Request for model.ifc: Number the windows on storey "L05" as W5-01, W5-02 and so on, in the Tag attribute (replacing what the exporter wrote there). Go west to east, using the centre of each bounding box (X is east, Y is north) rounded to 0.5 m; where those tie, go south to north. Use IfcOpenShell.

First a look at what the model holds.

```python
import ifcopenshell
import ifcopenshell.util.element
import ifcopenshell.util.placement

model = ifcopenshell.open("model.ifc")
print(model.schema)
storey = next(s for s in model.by_type("IfcBuildingStorey") if s.Name == "L05")
windows = [e for e in ifcopenshell.util.element.get_decomposition(storey) if e.is_a("IfcWindow")]
for e in sorted(windows, key=lambda e: e.id()):
    origin = ifcopenshell.util.placement.get_local_placement(e.ObjectPlacement)[:3, 3]
    print(e.id(), e.Tag, e.Name, origin.round(2) + 0.0, sep=" | ")
```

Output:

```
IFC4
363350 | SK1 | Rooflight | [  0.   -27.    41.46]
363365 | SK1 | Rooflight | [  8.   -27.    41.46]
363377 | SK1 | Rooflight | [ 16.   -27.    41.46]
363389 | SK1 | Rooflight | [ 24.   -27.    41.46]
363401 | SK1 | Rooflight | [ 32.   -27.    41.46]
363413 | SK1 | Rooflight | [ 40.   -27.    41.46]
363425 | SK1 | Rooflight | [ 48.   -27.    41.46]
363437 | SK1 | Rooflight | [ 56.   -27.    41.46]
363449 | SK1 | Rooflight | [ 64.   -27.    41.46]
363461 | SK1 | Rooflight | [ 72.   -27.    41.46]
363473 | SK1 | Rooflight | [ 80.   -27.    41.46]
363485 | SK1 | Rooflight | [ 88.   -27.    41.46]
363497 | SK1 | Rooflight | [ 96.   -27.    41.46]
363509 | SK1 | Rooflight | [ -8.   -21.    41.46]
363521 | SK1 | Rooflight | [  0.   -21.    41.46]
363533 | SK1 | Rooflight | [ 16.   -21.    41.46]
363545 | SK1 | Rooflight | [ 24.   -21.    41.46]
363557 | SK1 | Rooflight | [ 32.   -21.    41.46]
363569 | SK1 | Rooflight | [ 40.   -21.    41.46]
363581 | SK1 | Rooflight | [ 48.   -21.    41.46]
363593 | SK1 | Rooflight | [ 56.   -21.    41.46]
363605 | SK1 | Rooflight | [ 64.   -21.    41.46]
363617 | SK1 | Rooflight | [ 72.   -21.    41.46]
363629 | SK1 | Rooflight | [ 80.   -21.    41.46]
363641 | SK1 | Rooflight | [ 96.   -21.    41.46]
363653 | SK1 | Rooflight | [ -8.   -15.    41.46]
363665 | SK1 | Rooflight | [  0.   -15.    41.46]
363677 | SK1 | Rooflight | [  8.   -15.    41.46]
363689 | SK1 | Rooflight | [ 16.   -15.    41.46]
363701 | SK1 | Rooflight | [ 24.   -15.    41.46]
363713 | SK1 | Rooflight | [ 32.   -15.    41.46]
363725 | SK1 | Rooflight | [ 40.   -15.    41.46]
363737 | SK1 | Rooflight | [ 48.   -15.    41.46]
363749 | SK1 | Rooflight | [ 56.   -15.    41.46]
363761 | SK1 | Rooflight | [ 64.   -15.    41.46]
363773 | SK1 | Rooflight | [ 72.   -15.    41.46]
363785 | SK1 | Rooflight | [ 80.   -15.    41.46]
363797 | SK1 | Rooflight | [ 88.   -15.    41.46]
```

```python
import ifcopenshell
import ifcopenshell.geom
import ifcopenshell.util.element
import ifcopenshell.util.shape

model = ifcopenshell.open("model.ifc")
settings = ifcopenshell.geom.settings()
settings.set("use-world-coords", True)


def centre(element):
    shape = ifcopenshell.geom.create_shape(settings, element)
    return ifcopenshell.util.shape.get_bbox_centroid(shape.geometry)


storey = next(s for s in model.by_type("IfcBuildingStorey") if s.Name == "L05")
windows = [e for e in ifcopenshell.util.element.get_decomposition(storey) if e.is_a("IfcWindow")]

# Insertion points can sit at a corner or the storey origin, so sort by the geometry (in metres).
centres = {e: centre(e) for e in windows}
windows.sort(key=lambda e: (round(centres[e][0] / 0.5), centres[e][1]))

for i, e in enumerate(windows, start=1):
    number = f"W5-{i:02d}"
    e.Tag = number
    print(e.id(), number)

model.write("model_rev.ifc")
```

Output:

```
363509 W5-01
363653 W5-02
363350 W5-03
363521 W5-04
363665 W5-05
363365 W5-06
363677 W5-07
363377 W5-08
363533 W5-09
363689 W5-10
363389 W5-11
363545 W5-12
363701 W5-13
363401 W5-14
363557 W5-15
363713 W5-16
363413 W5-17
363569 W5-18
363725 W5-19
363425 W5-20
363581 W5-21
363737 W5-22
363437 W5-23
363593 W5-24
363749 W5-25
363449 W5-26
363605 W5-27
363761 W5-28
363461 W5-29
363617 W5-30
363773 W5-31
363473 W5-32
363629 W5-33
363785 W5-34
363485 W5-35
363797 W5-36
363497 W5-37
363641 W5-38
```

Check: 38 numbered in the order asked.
